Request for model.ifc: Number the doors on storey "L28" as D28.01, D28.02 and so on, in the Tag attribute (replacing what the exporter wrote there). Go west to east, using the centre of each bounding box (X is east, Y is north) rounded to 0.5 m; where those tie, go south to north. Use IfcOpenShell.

First a look at what the model holds.

```python
import ifcopenshell
import ifcopenshell.util.element
import ifcopenshell.util.placement

model = ifcopenshell.open("model.ifc")
print(model.schema)
storey = next(s for s in model.by_type("IfcBuildingStorey") if s.Name == "L28")
doors = [e for e in ifcopenshell.util.element.get_decomposition(storey) if e.is_a("IfcDoor")]
for e in sorted(doors, key=lambda e: e.id()):
    origin = ifcopenshell.util.placement.get_local_placement(e.ObjectPlacement)[:3, 3]
    print(e.id(), e.Tag, e.Name, origin.round(2) + 0.0, sep=" | ")
```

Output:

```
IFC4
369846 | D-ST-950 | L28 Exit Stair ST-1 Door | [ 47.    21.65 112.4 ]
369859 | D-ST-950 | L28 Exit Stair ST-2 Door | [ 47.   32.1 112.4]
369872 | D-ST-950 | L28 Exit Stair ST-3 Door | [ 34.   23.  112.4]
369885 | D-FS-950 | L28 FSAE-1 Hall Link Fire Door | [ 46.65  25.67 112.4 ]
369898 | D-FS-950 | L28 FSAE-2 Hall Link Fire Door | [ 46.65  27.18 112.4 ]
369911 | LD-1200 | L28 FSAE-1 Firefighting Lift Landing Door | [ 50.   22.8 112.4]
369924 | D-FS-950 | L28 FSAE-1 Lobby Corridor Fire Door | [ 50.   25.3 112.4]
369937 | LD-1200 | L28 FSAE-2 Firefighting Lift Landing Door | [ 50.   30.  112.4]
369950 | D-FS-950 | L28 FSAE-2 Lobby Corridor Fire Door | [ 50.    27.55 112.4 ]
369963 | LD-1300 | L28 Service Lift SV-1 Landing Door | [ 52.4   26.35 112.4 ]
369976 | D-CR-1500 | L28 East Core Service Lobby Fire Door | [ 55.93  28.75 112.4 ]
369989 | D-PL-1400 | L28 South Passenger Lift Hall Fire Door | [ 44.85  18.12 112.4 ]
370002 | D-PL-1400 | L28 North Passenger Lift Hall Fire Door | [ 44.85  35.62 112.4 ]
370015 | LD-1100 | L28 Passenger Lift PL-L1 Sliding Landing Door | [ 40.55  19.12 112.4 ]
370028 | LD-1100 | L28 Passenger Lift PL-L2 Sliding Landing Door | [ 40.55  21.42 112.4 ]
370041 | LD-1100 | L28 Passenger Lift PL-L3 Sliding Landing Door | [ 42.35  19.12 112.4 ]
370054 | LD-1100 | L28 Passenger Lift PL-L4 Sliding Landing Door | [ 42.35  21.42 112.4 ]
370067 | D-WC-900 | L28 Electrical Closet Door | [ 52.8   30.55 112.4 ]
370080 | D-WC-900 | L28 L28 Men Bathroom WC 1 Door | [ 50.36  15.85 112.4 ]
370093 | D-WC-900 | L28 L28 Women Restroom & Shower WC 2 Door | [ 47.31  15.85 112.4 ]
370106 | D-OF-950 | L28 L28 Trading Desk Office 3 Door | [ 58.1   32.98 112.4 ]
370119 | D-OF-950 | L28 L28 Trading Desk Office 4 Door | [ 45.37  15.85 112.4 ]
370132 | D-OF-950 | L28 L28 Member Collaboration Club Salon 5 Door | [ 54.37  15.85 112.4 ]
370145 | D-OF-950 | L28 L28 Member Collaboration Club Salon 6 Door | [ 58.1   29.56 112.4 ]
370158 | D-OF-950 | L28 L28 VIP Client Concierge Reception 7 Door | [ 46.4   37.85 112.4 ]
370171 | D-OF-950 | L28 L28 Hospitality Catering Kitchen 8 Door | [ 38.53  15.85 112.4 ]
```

```python
import ifcopenshell
import ifcopenshell.geom
import ifcopenshell.util.element
import ifcopenshell.util.shape

model = ifcopenshell.open("model.ifc")
settings = ifcopenshell.geom.settings()
settings.set("use-world-coords", True)


def centre(element):
    shape = ifcopenshell.geom.create_shape(settings, element)
    return ifcopenshell.util.shape.get_bbox_centroid(shape.geometry)


storey = next(s for s in model.by_type("IfcBuildingStorey") if s.Name == "L28")
doors = [e for e in ifcopenshell.util.element.get_decomposition(storey) if e.is_a("IfcDoor")]

# Insertion points can sit at a corner or the storey origin, so sort by the geometry (in metres).
centres = {e: centre(e) for e in doors}
doors.sort(key=lambda e: (round(centres[e][0] / 0.5), centres[e][1]))

for i, e in enumerate(doors, start=1):
    number = f"D28.{i:02d}"
    e.Tag = number
    print(e.id(), number)

model.write("model_v2.ifc")
```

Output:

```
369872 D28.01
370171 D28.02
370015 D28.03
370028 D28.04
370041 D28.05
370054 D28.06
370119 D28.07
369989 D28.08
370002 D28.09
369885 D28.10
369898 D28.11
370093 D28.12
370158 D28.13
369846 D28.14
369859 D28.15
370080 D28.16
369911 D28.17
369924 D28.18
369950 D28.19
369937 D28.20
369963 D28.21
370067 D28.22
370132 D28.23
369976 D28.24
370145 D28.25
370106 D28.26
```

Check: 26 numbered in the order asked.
